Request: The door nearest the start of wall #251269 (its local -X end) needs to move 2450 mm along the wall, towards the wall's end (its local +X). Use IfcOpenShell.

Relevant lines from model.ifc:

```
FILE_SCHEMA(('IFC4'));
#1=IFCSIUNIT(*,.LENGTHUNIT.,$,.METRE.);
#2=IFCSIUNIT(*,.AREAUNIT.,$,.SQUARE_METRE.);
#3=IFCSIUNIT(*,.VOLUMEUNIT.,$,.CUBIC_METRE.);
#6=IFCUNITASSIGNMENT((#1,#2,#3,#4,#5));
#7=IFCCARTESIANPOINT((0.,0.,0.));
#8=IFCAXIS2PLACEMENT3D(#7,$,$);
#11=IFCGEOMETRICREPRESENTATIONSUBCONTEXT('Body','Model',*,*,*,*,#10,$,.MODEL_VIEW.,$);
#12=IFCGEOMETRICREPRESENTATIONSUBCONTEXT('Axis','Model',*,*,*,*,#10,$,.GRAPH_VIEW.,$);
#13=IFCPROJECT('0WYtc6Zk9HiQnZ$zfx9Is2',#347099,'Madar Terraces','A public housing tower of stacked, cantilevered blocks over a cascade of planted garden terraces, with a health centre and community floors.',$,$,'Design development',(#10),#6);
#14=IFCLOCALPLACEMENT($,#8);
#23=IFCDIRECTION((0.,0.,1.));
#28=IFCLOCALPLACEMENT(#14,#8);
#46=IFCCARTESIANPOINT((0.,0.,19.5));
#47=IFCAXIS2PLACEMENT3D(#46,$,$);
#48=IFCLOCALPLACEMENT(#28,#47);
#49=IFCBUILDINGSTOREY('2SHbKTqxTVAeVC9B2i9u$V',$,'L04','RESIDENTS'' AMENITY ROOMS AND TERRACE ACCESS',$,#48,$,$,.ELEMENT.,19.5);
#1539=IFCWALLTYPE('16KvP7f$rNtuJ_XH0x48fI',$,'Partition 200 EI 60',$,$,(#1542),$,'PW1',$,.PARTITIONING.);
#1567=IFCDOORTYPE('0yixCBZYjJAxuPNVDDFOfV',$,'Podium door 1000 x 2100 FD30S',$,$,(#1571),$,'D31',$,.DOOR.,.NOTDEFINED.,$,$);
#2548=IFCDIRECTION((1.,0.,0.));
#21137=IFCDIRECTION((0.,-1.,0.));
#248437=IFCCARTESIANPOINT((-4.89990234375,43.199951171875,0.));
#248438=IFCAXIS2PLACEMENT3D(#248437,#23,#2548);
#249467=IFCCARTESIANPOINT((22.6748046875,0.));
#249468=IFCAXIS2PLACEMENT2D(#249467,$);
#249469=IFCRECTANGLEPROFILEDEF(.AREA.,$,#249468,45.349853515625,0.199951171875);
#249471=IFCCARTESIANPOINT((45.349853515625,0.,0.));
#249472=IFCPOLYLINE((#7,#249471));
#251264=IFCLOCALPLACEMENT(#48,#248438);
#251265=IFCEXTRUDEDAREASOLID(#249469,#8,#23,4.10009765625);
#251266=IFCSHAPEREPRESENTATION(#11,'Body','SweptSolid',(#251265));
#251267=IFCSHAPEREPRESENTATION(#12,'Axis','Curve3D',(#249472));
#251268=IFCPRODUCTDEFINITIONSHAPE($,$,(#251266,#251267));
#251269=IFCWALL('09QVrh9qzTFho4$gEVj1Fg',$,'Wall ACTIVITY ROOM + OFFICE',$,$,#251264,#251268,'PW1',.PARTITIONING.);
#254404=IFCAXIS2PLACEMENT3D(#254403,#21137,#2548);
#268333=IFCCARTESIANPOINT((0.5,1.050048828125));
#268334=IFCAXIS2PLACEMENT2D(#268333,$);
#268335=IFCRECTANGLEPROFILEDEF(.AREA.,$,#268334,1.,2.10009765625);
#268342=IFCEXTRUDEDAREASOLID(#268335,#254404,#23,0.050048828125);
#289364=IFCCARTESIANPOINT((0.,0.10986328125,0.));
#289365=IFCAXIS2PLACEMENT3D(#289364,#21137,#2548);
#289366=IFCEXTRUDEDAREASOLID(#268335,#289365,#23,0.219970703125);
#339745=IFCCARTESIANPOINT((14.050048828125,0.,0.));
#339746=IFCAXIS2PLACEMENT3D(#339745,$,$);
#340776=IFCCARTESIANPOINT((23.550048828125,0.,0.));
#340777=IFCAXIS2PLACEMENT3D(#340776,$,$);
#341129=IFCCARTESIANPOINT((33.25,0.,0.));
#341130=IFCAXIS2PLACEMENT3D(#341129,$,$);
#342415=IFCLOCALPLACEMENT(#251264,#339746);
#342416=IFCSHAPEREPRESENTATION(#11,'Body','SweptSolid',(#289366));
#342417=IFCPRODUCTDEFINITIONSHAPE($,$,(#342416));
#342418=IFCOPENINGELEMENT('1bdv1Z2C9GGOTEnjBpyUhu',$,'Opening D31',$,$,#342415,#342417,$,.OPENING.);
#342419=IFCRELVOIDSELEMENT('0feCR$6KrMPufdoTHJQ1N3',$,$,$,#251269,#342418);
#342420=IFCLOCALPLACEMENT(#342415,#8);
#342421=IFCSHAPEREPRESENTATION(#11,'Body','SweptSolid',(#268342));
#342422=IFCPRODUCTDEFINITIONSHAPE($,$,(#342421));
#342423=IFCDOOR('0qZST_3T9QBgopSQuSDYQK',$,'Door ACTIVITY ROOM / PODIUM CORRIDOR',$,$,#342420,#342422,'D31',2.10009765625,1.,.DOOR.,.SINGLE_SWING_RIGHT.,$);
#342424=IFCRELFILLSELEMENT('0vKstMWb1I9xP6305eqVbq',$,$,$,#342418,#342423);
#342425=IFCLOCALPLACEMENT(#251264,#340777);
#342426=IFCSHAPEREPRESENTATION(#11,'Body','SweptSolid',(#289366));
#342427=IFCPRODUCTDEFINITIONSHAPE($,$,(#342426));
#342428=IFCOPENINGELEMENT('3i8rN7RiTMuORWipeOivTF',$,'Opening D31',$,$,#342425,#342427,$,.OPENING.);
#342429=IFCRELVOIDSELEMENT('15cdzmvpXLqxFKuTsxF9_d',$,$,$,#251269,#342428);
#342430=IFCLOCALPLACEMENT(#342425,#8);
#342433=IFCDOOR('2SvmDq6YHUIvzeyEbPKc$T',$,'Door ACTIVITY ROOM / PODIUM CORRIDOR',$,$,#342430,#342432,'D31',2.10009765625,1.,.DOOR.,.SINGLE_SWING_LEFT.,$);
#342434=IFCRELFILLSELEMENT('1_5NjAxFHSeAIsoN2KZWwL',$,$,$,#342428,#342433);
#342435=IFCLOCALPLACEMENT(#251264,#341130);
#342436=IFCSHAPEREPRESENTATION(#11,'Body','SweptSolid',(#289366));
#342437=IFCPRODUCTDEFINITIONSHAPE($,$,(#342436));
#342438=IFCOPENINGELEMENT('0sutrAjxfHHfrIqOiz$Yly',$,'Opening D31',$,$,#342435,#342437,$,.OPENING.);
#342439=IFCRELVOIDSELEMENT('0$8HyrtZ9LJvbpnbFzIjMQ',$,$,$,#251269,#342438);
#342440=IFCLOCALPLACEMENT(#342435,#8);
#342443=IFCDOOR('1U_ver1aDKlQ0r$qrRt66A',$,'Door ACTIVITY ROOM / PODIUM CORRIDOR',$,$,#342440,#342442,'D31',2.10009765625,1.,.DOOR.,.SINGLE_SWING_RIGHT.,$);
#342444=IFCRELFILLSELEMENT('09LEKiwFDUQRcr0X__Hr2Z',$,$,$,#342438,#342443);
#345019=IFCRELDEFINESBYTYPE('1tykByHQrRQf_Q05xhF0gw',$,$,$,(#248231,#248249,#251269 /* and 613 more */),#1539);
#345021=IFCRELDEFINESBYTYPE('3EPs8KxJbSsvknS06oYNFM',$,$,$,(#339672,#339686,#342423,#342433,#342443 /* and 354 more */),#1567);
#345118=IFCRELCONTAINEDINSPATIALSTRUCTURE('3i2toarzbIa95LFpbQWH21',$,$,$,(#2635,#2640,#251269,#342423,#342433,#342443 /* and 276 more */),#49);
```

```python
import ifcopenshell
import ifcopenshell.api.geometry
import ifcopenshell.util.placement

model = ifcopenshell.open("model.ifc")

door = model.by_guid("0qZST_3T9QBgopSQuSDYQK")
opening = door.FillsVoids[0].RelatingOpeningElement
wall = opening.VoidsElements[0].RelatingBuildingElement

wall_matrix = ifcopenshell.util.placement.get_local_placement(wall.ObjectPlacement)
shift = wall_matrix[:3, 0] * 2.45
before = ifcopenshell.util.placement.get_local_placement(door.ObjectPlacement)[:3, 3].copy()

# The door is placed relative to its opening, so it follows when the opening moves.
matrix = ifcopenshell.util.placement.get_local_placement(opening.ObjectPlacement)
matrix[:3, 3] += shift
ifcopenshell.api.geometry.edit_object_placement(
    model, product=opening, matrix=matrix, is_si=False, should_transform_children=True
)

after = ifcopenshell.util.placement.get_local_placement(door.ObjectPlacement)[:3, 3]
print("door moved by", (after - before).round(3) + 0.0)

model.write("model_v2.ifc")
```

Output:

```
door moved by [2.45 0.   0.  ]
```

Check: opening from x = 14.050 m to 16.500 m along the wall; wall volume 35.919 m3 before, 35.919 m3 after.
